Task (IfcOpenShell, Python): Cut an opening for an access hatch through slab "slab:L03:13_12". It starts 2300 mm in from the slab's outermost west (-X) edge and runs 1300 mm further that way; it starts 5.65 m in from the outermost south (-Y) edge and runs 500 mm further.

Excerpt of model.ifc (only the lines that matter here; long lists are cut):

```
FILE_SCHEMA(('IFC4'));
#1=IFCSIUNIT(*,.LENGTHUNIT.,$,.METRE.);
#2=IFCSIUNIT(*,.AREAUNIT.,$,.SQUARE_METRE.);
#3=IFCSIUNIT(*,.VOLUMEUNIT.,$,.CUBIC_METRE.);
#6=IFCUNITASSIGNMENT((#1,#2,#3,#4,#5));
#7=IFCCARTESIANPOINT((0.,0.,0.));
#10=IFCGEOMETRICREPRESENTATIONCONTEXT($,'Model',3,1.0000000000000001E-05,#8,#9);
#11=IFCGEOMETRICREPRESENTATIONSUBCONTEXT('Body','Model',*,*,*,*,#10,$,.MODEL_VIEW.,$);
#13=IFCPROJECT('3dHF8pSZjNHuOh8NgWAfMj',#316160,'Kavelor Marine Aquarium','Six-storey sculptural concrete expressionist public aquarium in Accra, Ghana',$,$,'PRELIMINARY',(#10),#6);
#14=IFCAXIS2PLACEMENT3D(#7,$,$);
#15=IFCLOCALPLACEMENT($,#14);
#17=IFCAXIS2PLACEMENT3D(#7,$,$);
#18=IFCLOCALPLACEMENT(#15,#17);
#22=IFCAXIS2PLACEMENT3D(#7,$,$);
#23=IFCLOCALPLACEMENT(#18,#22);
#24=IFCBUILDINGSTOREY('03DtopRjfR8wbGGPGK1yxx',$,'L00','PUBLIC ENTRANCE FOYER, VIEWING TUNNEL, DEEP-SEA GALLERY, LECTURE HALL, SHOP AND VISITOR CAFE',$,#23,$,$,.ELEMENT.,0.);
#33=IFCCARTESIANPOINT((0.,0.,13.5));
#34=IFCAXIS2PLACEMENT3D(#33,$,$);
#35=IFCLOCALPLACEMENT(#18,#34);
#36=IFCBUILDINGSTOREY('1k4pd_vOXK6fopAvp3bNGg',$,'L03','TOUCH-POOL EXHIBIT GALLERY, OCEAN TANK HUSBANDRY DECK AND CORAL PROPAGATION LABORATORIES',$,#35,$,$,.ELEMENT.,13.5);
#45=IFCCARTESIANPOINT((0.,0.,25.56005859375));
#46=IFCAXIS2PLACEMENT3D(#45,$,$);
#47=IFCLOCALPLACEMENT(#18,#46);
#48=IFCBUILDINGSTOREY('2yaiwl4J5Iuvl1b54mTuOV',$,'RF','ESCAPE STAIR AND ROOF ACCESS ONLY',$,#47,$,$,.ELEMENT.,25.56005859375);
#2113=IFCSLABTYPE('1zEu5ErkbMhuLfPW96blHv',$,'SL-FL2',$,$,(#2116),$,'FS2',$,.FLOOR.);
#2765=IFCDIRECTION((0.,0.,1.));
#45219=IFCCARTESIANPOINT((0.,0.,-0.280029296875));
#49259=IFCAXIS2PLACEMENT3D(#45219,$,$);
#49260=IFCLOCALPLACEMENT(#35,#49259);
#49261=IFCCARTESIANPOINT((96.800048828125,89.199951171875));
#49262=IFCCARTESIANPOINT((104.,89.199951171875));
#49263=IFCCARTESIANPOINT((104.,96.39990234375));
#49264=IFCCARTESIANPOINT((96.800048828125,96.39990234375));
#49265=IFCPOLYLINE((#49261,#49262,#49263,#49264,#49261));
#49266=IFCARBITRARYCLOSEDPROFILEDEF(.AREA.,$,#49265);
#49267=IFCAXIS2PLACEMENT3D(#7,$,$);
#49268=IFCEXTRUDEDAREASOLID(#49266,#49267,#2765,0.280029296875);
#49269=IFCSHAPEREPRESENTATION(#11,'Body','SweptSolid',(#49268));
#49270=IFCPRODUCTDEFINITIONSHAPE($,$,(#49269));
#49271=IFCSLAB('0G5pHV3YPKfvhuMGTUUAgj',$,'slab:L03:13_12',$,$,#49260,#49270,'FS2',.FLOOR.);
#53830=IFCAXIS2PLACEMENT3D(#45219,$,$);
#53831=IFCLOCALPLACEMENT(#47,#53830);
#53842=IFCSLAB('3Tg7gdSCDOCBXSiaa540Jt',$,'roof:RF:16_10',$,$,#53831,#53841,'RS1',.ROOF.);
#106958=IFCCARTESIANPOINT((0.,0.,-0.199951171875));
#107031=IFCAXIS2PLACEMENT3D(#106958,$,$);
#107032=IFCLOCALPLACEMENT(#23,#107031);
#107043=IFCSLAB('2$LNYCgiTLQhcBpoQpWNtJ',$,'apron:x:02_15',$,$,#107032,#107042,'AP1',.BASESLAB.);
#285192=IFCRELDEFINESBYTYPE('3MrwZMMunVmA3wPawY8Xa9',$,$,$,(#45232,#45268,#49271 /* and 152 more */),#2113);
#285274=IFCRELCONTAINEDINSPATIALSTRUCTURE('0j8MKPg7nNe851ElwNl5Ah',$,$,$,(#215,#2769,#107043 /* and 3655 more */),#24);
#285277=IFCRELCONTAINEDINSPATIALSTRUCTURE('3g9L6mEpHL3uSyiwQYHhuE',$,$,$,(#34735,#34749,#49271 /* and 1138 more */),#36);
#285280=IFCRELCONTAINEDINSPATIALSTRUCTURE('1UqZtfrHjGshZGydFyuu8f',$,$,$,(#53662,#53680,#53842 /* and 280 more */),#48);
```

```python
import numpy as np
import ifcopenshell
import ifcopenshell.api.feature
import ifcopenshell.api.geometry
import ifcopenshell.api.root
import ifcopenshell.geom
import ifcopenshell.util.placement
import ifcopenshell.util.representation
import ifcopenshell.util.shape
import ifcopenshell.util.unit

model = ifcopenshell.open("model.ifc")
unit_scale = ifcopenshell.util.unit.calculate_unit_scale(model)
settings = ifcopenshell.geom.settings()


def volume(element):
    """Net volume in cubic metres, openings subtracted."""
    shape = ifcopenshell.geom.create_shape(settings, element)
    return ifcopenshell.util.shape.get_volume(shape.geometry)


slab = model.by_id(49271)
before = volume(slab)

# Extent in the slab's own axes, in metres. The edges named are its -X and -Y sides.
slab_shape = ifcopenshell.geom.create_shape(settings, slab)
vertices = ifcopenshell.util.shape.get_vertices(slab_shape.geometry)
x_min, y_min, bottom = vertices.min(axis=0)
top = vertices[:, 2].max()

opening = ifcopenshell.api.root.create_entity(model, ifc_class="IfcOpeningElement", name="Access hatch opening", predefined_type="OPENING")
context = ifcopenshell.util.representation.get_context(model, "Model", "Body", "MODEL_VIEW")
width, depth = 1.3, 0.5
outline = [(0.0, 0.0), (width, 0.0), (width, depth), (0.0, depth), (0.0, 0.0)]
# Overshoot both faces by 50 mm so the cut is clean.
shape = ifcopenshell.api.geometry.add_slab_representation(
    model, context=context, depth=top - bottom + 0.1, polyline=outline
)
ifcopenshell.api.geometry.assign_representation(model, product=opening, representation=shape)

matrix = ifcopenshell.util.placement.get_local_placement(slab.ObjectPlacement)
matrix[:, 3] = matrix @ np.append(np.array([x_min + 2.3, y_min + 5.65, bottom - 0.05]) / unit_scale, 1.0)
ifcopenshell.api.geometry.edit_object_placement(model, product=opening, matrix=matrix, is_si=False)
ifcopenshell.api.feature.add_feature(model, feature=opening, element=slab)

after = volume(slab)

print(f"slab volume {before:.3f} -> {after:.3f} m3")

model.write("model-out.ifc")
```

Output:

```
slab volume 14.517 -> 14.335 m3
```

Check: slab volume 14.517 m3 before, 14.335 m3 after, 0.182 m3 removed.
